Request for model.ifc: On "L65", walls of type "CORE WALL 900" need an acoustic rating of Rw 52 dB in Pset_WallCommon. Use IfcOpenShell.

First a look at what the model holds.

```python
import ifcopenshell
import ifcopenshell.util.element

model = ifcopenshell.open("model.ifc")
print(model.schema)
storey = next(s for s in model.by_type("IfcBuildingStorey") if s.Name == "L65")
walls = [e for e in ifcopenshell.util.element.get_decomposition(storey) if e.is_a("IfcWall")]
seen = {}
for e in walls:
    element_type = ifcopenshell.util.element.get_type(e)
    key = (element_type.Name if element_type != e and element_type else None, ifcopenshell.util.element.get_pset(e, "Pset_WallCommon", "AcousticRating"))
    seen[key] = seen.get(key, 0) + 1
for (name, value), count in sorted(seen.items(), key=str):
    print(count, "x", name, "|", value)
```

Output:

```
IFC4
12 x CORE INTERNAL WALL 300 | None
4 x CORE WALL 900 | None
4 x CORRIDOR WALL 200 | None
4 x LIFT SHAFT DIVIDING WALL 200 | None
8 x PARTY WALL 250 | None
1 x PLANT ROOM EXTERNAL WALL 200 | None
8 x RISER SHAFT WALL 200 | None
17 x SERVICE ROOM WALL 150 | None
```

```python
import ifcopenshell
import ifcopenshell.api.pset
import ifcopenshell.util.element

model = ifcopenshell.open("model.ifc")

storey = next(s for s in model.by_type("IfcBuildingStorey") if s.Name == "L65")
walls = [e for e in ifcopenshell.util.element.get_decomposition(storey) if e.is_a("IfcWall")]

count = 0
for e in walls:
    element_type = ifcopenshell.util.element.get_type(e)
    if element_type in (None, e) or element_type.Name != "CORE WALL 900":
        continue
    found = ifcopenshell.util.element.get_pset(e, "Pset_WallCommon", should_inherit=False)
    if found:
        pset = model.by_id(found["id"])
        if len(ifcopenshell.util.element.get_elements_by_pset(pset)) > 1:
            pset = ifcopenshell.api.pset.unshare_pset(model, products=[e], pset=pset)[0]
    else:
        pset = ifcopenshell.api.pset.add_pset(model, product=e, name="Pset_WallCommon")
    ifcopenshell.api.pset.edit_pset(model, pset=pset, properties={"AcousticRating": "Rw 52 dB"})
    count += 1

print(count, "walls updated")

model.write("model_rev.ifc")
```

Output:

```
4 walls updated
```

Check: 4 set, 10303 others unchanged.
